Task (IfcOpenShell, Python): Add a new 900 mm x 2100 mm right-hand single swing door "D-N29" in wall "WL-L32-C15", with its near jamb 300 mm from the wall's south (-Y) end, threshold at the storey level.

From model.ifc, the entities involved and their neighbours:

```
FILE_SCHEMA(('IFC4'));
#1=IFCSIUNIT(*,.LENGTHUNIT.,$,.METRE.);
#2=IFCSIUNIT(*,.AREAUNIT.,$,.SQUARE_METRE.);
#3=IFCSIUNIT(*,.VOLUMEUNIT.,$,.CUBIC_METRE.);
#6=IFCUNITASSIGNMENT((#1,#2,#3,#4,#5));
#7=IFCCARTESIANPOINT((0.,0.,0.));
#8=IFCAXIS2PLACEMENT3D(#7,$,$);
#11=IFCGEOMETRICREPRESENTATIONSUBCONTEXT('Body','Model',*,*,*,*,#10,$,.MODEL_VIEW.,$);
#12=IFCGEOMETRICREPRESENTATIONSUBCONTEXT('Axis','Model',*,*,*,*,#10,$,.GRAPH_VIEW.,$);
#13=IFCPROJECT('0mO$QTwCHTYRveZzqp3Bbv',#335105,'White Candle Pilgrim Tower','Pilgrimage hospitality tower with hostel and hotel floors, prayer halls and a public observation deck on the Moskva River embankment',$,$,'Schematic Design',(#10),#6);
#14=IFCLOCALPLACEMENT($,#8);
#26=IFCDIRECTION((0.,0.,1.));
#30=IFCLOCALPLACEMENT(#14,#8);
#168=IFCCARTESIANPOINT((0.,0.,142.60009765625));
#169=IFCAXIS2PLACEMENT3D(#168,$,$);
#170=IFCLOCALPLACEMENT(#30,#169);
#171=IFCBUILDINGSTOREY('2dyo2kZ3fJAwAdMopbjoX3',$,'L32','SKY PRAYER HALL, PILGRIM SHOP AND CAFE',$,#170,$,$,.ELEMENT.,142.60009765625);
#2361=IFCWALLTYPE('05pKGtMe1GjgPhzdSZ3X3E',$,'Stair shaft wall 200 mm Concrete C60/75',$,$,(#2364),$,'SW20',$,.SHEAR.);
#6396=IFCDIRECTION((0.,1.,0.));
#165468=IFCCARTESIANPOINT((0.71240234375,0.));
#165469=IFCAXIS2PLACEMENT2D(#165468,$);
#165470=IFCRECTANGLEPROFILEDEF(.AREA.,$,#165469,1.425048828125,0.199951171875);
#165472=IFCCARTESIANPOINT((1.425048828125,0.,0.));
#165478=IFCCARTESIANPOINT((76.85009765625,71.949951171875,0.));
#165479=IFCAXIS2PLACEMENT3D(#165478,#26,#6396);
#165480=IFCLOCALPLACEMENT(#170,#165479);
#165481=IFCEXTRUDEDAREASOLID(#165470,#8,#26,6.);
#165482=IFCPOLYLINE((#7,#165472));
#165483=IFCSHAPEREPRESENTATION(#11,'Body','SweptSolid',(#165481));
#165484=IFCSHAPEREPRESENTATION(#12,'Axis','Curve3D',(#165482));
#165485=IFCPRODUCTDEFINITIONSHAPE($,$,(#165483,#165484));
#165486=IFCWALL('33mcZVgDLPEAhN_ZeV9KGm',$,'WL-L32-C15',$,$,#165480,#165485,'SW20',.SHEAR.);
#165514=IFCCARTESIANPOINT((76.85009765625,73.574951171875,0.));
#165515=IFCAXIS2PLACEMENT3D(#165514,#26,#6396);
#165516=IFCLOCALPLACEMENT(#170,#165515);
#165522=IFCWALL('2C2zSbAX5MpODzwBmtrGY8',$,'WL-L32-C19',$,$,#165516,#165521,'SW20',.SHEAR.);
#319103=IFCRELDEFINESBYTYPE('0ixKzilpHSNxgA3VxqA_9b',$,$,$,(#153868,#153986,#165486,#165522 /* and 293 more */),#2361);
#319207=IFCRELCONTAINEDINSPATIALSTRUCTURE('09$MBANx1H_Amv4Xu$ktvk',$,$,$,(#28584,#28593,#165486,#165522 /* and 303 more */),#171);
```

```python
import numpy as np
import ifcopenshell
import ifcopenshell.api.feature
import ifcopenshell.api.geometry
import ifcopenshell.api.root
import ifcopenshell.api.spatial
import ifcopenshell.geom
import ifcopenshell.util.element
import ifcopenshell.util.placement
import ifcopenshell.util.representation
import ifcopenshell.util.shape
import ifcopenshell.util.unit

model = ifcopenshell.open("model.ifc")
unit_scale = ifcopenshell.util.unit.calculate_unit_scale(model)
settings = ifcopenshell.geom.settings()


def volume(element):
    """Net volume in cubic metres, openings subtracted."""
    shape = ifcopenshell.geom.create_shape(settings, element)
    return ifcopenshell.util.shape.get_volume(shape.geometry)


wall = model.by_guid("33mcZVgDLPEAhN_ZeV9KGm")
storey = ifcopenshell.util.element.get_container(wall, ifc_class="IfcBuildingStorey")
context = ifcopenshell.util.representation.get_context(model, "Model", "Body", "MODEL_VIEW")
before = volume(wall)

width, height, from_end, sill = 0.9, 2.1, 0.3, 0.0  # metres

# The wall runs along its own X axis, and the end named is its -X end.
wall_shape = ifcopenshell.geom.create_shape(settings, wall)
x, y, z = ifcopenshell.util.shape.get_vertices(wall_shape.geometry).T
start = x.min() + from_end
face, thickness = float(y.min()), float(y.max() - y.min())
wall_matrix = ifcopenshell.util.placement.get_local_placement(wall.ObjectPlacement)
level = ifcopenshell.util.placement.get_local_placement(storey.ObjectPlacement)[2, 3]


def in_wall(x, y):
    """Placement at x, y metres in the wall's axes, at sill height."""
    matrix = wall_matrix.copy()
    matrix[:, 3] = wall_matrix @ np.array([x / unit_scale, y / unit_scale, 0.0, 1.0])
    matrix[2, 3] = level + sill / unit_scale
    return matrix


# Opening: a box that overshoots both wall faces by 50 mm.
opening = ifcopenshell.api.root.create_entity(model, ifc_class="IfcOpeningElement", predefined_type="OPENING")
box = ifcopenshell.api.geometry.add_wall_representation(
    model, context=context, length=width, height=height, thickness=thickness + 0.1
)
ifcopenshell.api.geometry.assign_representation(model, product=opening, representation=box)
ifcopenshell.api.geometry.edit_object_placement(model, product=opening, matrix=in_wall(start, face - 0.05), is_si=False)
ifcopenshell.api.feature.add_feature(model, feature=opening, element=wall)

door = ifcopenshell.api.root.create_entity(model, ifc_class="IfcDoor", name="D-N29", predefined_type="DOOR")
door.OverallWidth, door.OverallHeight = width / unit_scale, height / unit_scale
door.OperationType = "SINGLE_SWING_RIGHT"
body = ifcopenshell.api.geometry.add_door_representation(
    model,
    context=context,
    overall_width=door.OverallWidth,
    overall_height=door.OverallHeight,
    operation_type="SINGLE_SWING_RIGHT",
    lining_properties={"LiningDepth": thickness / unit_scale, "ThresholdDepth": thickness / unit_scale},
)
ifcopenshell.api.geometry.assign_representation(model, product=door, representation=body)
ifcopenshell.api.spatial.assign_container(model, products=[door], relating_structure=storey)
ifcopenshell.api.feature.add_filling(model, opening=opening, element=door)

# The lining spans the wall, so the door starts at the wall face.
ifcopenshell.api.geometry.edit_object_placement(model, product=door, matrix=in_wall(start, face), is_si=False)

after = volume(wall)

print(f"wall volume {before:.3f} -> {after:.3f} m3")

model.write("model_v2.ifc")
```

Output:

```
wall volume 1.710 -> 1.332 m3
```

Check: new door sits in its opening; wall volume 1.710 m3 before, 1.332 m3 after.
